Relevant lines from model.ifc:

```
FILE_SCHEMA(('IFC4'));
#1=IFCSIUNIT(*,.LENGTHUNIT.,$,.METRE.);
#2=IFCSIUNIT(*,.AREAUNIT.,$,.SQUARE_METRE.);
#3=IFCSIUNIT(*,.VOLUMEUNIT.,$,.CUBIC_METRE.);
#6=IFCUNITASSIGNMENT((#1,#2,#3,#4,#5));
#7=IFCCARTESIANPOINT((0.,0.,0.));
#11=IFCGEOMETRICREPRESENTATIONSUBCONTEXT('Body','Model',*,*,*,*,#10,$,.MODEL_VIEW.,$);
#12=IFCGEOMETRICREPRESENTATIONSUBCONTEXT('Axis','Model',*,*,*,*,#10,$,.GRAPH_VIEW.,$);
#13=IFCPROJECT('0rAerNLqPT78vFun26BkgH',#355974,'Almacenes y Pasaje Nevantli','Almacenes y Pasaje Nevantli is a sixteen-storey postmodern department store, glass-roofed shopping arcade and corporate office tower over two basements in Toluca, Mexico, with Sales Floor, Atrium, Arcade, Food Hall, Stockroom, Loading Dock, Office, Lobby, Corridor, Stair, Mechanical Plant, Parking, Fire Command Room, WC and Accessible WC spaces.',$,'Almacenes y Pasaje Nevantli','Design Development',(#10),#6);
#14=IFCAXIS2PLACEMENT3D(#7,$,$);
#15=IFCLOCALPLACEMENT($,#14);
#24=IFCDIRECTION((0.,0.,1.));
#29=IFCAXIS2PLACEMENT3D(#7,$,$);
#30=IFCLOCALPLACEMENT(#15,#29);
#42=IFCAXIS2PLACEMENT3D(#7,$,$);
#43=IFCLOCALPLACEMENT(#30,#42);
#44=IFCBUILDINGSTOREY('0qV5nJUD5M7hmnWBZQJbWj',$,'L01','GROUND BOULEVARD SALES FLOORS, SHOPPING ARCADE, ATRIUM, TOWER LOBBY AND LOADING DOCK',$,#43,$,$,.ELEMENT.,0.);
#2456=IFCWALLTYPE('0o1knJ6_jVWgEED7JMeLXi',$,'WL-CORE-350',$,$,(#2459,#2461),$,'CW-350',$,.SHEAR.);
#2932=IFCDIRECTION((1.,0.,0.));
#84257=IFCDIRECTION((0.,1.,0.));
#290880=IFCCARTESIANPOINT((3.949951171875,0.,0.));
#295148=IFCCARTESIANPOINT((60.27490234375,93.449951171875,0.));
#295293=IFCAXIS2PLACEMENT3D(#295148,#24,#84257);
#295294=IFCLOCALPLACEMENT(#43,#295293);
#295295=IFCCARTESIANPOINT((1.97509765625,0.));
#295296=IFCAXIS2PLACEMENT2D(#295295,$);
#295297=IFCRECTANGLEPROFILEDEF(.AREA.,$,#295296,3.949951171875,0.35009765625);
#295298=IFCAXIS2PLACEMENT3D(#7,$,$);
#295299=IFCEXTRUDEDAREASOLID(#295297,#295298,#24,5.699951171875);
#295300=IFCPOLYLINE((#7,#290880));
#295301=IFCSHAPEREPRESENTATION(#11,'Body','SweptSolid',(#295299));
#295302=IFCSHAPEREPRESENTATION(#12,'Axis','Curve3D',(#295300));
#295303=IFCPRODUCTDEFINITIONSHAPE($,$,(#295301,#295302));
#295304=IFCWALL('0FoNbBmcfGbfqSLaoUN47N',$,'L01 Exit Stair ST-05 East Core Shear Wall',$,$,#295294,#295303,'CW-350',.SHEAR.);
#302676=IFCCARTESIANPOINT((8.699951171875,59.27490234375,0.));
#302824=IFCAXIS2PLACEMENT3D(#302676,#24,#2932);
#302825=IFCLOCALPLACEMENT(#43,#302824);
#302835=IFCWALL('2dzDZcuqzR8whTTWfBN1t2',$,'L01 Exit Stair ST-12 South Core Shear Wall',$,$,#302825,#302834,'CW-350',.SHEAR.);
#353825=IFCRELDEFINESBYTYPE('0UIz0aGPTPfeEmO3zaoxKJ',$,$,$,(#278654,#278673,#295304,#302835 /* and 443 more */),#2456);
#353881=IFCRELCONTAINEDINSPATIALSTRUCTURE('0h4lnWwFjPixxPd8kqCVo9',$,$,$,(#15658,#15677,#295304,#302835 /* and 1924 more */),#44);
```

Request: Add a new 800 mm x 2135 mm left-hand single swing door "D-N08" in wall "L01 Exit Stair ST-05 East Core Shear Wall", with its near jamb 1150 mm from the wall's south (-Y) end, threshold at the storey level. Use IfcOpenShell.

```python
import numpy as np
import ifcopenshell
import ifcopenshell.api.feature
import ifcopenshell.api.geometry
import ifcopenshell.api.root
import ifcopenshell.api.spatial
import ifcopenshell.geom
import ifcopenshell.util.element
import ifcopenshell.util.placement
import ifcopenshell.util.representation
import ifcopenshell.util.shape
import ifcopenshell.util.unit

model = ifcopenshell.open("model.ifc")
unit_scale = ifcopenshell.util.unit.calculate_unit_scale(model)
settings = ifcopenshell.geom.settings()


def volume(element):
    """Net volume in cubic metres, openings subtracted."""
    shape = ifcopenshell.geom.create_shape(settings, element)
    return ifcopenshell.util.shape.get_volume(shape.geometry)


wall = model.by_guid("0FoNbBmcfGbfqSLaoUN47N")
storey = ifcopenshell.util.element.get_container(wall, ifc_class="IfcBuildingStorey")
context = ifcopenshell.util.representation.get_context(model, "Model", "Body", "MODEL_VIEW")
before = volume(wall)

width, height, from_end, sill = 0.8, 2.135, 1.15, 0.0  # metres

# The wall runs along its own X axis, and the end named is its -X end.
wall_shape = ifcopenshell.geom.create_shape(settings, wall)
x, y, z = ifcopenshell.util.shape.get_vertices(wall_shape.geometry).T
start = x.min() + from_end
face, thickness = float(y.min()), float(y.max() - y.min())
wall_matrix = ifcopenshell.util.placement.get_local_placement(wall.ObjectPlacement)
level = ifcopenshell.util.placement.get_local_placement(storey.ObjectPlacement)[2, 3]


def in_wall(x, y):
    """Placement at x, y metres in the wall's axes, at sill height."""
    matrix = wall_matrix.copy()
    matrix[:, 3] = wall_matrix @ np.array([x / unit_scale, y / unit_scale, 0.0, 1.0])
    matrix[2, 3] = level + sill / unit_scale
    return matrix


# Opening: a box that overshoots both wall faces by 50 mm.
opening = ifcopenshell.api.root.create_entity(model, ifc_class="IfcOpeningElement", predefined_type="OPENING")
box = ifcopenshell.api.geometry.add_wall_representation(
    model, context=context, length=width, height=height, thickness=thickness + 0.1
)
ifcopenshell.api.geometry.assign_representation(model, product=opening, representation=box)
ifcopenshell.api.geometry.edit_object_placement(model, product=opening, matrix=in_wall(start, face - 0.05), is_si=False)
ifcopenshell.api.feature.add_feature(model, feature=opening, element=wall)

door = ifcopenshell.api.root.create_entity(model, ifc_class="IfcDoor", name="D-N08", predefined_type="DOOR")
door.OverallWidth, door.OverallHeight = width / unit_scale, height / unit_scale
door.OperationType = "SINGLE_SWING_LEFT"
body = ifcopenshell.api.geometry.add_door_representation(
    model,
    context=context,
    overall_width=door.OverallWidth,
    overall_height=door.OverallHeight,
    operation_type="SINGLE_SWING_LEFT",
    lining_properties={"LiningDepth": thickness / unit_scale, "ThresholdDepth": thickness / unit_scale},
)
ifcopenshell.api.geometry.assign_representation(model, product=door, representation=body)
ifcopenshell.api.spatial.assign_container(model, products=[door], relating_structure=storey)
ifcopenshell.api.feature.add_filling(model, opening=opening, element=door)

# The lining spans the wall, so the door starts at the wall face.
ifcopenshell.api.geometry.edit_object_placement(model, product=door, matrix=in_wall(start, face), is_si=False)

after = volume(wall)

print(f"wall volume {before:.3f} -> {after:.3f} m3")

model.write("model-out.ifc")
```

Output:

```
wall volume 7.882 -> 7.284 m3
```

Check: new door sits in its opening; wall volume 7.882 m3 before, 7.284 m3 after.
